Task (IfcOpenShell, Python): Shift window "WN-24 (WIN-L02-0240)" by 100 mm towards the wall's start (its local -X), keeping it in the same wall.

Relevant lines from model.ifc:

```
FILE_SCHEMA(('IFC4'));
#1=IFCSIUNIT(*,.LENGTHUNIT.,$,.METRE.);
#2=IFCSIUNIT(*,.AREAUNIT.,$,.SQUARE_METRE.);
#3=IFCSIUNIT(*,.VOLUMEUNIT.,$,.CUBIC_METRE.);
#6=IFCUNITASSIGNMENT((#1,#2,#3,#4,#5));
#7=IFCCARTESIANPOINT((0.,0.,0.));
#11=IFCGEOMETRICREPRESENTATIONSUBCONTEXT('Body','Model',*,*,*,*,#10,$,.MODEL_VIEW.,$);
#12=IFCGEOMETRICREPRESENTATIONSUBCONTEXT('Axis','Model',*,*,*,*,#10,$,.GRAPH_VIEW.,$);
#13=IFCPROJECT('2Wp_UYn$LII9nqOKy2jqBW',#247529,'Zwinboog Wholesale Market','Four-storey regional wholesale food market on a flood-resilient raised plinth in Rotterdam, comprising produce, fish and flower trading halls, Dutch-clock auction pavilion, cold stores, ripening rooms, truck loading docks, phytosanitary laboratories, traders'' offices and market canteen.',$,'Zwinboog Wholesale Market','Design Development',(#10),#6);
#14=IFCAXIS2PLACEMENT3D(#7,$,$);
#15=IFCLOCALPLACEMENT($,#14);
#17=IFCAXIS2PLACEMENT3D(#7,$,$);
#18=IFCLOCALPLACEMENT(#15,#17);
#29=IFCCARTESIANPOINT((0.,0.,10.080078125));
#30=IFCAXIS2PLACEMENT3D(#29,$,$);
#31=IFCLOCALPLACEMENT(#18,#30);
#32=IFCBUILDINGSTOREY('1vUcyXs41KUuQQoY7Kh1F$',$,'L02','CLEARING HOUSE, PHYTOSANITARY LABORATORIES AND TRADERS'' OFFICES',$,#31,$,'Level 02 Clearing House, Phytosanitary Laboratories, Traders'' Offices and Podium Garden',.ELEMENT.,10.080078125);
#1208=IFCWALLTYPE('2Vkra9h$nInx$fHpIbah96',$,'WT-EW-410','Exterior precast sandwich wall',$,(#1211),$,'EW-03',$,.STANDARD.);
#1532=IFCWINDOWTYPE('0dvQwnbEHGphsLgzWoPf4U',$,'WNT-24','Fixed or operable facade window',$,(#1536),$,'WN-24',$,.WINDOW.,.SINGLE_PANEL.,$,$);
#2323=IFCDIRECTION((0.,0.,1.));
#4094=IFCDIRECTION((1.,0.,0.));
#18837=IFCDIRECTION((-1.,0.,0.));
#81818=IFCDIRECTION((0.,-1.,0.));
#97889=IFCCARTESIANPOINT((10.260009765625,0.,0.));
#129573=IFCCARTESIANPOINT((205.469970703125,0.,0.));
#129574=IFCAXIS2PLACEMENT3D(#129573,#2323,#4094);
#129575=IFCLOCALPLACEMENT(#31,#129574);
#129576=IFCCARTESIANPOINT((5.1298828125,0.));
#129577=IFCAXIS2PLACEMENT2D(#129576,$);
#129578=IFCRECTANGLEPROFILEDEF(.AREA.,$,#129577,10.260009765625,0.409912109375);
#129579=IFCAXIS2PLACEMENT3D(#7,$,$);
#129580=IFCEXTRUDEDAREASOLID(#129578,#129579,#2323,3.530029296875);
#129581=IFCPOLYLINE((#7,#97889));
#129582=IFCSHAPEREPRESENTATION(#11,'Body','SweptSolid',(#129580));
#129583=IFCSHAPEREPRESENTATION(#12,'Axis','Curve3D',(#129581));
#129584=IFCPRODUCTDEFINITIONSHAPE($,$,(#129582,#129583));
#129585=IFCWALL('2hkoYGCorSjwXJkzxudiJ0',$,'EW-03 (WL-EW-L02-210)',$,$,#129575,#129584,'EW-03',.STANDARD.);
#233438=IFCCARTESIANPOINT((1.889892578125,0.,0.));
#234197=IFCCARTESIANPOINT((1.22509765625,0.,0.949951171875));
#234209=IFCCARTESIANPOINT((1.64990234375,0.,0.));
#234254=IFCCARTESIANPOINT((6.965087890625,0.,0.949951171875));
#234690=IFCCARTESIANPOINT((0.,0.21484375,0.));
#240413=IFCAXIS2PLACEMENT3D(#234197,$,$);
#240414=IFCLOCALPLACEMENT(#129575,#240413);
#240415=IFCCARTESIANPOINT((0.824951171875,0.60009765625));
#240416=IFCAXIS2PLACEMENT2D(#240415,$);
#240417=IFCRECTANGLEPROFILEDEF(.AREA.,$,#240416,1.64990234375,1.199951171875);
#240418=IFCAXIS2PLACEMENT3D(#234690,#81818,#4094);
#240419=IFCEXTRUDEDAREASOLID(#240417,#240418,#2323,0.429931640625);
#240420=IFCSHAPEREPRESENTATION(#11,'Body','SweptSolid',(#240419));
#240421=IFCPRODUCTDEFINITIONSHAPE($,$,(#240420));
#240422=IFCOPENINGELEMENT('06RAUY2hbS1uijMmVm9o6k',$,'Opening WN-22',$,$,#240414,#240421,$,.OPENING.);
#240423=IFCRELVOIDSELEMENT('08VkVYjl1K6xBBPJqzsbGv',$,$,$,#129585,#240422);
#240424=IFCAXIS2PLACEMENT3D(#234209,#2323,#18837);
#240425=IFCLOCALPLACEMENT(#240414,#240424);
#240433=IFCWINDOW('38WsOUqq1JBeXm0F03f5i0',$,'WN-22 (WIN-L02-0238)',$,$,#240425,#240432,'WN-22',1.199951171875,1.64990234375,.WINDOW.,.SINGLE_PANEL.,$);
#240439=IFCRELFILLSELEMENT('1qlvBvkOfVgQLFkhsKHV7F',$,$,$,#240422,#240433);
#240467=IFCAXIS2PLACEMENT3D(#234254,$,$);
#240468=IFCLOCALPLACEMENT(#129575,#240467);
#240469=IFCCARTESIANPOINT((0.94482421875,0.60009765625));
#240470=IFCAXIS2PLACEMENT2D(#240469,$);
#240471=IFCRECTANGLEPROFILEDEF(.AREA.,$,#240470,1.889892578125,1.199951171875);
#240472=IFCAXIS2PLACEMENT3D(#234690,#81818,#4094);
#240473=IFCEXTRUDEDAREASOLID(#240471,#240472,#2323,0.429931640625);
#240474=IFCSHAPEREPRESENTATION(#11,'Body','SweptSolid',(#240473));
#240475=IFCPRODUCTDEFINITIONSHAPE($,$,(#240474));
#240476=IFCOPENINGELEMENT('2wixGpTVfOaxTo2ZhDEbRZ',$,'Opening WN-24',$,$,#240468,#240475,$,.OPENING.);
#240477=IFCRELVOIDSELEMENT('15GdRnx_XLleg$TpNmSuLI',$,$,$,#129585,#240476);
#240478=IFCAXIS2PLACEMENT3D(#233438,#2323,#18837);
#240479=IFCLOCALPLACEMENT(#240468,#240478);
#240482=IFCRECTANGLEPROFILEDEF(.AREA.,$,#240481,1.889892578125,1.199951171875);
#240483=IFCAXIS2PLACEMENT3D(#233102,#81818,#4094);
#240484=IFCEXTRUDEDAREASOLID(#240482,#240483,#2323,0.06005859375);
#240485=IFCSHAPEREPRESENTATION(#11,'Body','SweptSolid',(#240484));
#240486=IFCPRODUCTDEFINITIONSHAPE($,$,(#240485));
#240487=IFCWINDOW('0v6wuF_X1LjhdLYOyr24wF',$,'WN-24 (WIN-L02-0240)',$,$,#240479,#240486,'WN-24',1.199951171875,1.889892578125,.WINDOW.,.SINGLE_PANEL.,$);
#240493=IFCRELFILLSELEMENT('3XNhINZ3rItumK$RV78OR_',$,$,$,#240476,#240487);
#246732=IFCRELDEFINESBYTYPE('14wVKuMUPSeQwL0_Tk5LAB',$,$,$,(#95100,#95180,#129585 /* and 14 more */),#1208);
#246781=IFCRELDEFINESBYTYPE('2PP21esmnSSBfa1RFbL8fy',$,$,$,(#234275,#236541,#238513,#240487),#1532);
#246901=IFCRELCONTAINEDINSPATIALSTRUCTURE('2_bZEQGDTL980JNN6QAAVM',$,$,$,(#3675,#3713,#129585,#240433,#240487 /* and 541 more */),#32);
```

```python
import ifcopenshell
import ifcopenshell.api.geometry
import ifcopenshell.util.placement

model = ifcopenshell.open("model.ifc")

window = model.by_guid("0v6wuF_X1LjhdLYOyr24wF")
opening = window.FillsVoids[0].RelatingOpeningElement
wall = opening.VoidsElements[0].RelatingBuildingElement

wall_matrix = ifcopenshell.util.placement.get_local_placement(wall.ObjectPlacement)
shift = wall_matrix[:3, 0] * -0.1
before = ifcopenshell.util.placement.get_local_placement(window.ObjectPlacement)[:3, 3].copy()

# The window is placed relative to its opening, so it follows when the opening moves.
matrix = ifcopenshell.util.placement.get_local_placement(opening.ObjectPlacement)
matrix[:3, 3] += shift
ifcopenshell.api.geometry.edit_object_placement(
    model, product=opening, matrix=matrix, is_si=False, should_transform_children=True
)

after = ifcopenshell.util.placement.get_local_placement(window.ObjectPlacement)[:3, 3]
print("window moved by", (after - before).round(3) + 0.0)

model.write("model-out.ifc")
```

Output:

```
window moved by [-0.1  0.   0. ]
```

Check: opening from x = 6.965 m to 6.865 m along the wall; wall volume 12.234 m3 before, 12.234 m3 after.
